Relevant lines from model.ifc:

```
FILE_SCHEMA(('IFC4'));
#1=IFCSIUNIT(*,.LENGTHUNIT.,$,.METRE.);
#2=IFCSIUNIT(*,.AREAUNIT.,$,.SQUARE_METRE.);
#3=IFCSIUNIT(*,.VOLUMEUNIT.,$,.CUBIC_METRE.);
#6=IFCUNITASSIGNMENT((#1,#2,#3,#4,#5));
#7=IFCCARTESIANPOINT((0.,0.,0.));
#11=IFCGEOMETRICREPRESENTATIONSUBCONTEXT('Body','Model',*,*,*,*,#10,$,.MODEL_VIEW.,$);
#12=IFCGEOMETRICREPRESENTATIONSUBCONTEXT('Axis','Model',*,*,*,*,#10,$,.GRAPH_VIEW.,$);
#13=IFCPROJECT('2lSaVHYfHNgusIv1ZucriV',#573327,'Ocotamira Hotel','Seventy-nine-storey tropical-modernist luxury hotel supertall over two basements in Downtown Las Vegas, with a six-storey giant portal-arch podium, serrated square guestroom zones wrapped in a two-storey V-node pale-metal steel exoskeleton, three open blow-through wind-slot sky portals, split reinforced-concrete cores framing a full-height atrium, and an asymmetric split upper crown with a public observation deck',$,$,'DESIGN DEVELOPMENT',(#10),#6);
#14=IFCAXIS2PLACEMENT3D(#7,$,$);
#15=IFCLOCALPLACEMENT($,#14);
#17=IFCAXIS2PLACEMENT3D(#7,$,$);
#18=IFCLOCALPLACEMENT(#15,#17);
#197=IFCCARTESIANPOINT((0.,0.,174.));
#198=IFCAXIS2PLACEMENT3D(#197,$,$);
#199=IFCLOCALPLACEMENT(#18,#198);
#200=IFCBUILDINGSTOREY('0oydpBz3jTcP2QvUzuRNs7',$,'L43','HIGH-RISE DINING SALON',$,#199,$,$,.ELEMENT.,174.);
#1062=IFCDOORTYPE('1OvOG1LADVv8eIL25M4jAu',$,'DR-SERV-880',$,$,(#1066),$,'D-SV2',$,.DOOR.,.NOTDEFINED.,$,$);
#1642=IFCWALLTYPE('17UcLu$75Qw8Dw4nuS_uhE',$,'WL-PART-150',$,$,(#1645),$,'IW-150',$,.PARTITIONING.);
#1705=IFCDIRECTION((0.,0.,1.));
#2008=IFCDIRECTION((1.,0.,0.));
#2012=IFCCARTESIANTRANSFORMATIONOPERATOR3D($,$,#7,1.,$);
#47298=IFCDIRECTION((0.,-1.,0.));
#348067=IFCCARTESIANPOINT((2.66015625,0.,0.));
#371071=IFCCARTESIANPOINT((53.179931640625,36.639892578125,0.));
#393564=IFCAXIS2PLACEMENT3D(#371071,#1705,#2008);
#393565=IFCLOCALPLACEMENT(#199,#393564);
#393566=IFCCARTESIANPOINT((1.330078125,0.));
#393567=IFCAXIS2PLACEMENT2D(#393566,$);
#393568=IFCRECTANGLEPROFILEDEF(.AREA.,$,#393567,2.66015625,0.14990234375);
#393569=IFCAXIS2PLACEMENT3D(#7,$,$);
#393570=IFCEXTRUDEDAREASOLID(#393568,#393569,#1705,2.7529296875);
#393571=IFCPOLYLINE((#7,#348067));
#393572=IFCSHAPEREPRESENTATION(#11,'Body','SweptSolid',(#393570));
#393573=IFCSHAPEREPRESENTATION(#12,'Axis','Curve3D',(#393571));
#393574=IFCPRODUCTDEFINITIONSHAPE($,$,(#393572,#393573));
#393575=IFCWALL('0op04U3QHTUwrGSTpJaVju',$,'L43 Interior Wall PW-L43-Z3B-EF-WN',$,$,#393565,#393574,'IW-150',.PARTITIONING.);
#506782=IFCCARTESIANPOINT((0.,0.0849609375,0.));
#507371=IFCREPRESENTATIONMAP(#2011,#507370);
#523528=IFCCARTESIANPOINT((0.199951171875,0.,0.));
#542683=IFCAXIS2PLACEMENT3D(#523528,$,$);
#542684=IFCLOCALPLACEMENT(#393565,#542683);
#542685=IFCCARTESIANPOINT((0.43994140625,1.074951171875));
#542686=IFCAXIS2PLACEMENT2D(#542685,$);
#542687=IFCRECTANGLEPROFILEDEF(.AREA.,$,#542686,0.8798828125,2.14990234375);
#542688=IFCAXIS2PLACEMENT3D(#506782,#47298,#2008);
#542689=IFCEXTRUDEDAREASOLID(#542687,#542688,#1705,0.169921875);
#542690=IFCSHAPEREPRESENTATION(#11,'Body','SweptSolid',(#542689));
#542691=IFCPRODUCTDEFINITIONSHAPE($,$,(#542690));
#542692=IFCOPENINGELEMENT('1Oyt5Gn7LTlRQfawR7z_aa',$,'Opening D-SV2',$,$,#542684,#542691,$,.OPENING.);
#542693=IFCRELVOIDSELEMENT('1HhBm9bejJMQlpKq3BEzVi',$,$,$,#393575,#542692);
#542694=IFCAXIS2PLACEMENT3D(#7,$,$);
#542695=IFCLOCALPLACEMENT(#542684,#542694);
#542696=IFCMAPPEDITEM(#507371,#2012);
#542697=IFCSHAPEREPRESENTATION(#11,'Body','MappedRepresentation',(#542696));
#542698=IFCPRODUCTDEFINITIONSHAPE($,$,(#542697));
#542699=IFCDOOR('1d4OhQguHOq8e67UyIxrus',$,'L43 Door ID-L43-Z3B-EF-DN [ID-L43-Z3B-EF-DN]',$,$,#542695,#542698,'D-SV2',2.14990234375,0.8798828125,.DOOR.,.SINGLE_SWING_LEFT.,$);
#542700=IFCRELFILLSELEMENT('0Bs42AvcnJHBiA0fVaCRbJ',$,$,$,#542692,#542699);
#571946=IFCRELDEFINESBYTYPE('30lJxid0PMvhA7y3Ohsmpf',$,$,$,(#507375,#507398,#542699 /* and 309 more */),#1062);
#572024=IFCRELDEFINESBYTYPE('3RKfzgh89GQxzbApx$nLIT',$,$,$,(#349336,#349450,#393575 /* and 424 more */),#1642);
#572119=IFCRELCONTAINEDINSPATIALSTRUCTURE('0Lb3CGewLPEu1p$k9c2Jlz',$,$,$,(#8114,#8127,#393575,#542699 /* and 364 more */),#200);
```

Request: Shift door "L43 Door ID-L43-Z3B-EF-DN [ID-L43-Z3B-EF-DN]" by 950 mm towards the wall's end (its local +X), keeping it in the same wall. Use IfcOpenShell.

```python
import ifcopenshell
import ifcopenshell.api.geometry
import ifcopenshell.util.placement
import ifcopenshell.util.unit

model = ifcopenshell.open("model.ifc")
unit_scale = ifcopenshell.util.unit.calculate_unit_scale(model)

door = model.by_id(542699)
opening = door.FillsVoids[0].RelatingOpeningElement
wall = opening.VoidsElements[0].RelatingBuildingElement

wall_matrix = ifcopenshell.util.placement.get_local_placement(wall.ObjectPlacement)
shift = wall_matrix[:3, 0] * 0.95 / unit_scale
before = ifcopenshell.util.placement.get_local_placement(door.ObjectPlacement)[:3, 3].copy()

# The door is placed relative to its opening, so it follows when the opening moves.
matrix = ifcopenshell.util.placement.get_local_placement(opening.ObjectPlacement)
matrix[:3, 3] += shift
ifcopenshell.api.geometry.edit_object_placement(
    model, product=opening, matrix=matrix, is_si=False, should_transform_children=True
)

after = ifcopenshell.util.placement.get_local_placement(door.ObjectPlacement)[:3, 3]
print("door moved by", (after - before).round(3) + 0.0)

model.write("model_v2.ifc")
```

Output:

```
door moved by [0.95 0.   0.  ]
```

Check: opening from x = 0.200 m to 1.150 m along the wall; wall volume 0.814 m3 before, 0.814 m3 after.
